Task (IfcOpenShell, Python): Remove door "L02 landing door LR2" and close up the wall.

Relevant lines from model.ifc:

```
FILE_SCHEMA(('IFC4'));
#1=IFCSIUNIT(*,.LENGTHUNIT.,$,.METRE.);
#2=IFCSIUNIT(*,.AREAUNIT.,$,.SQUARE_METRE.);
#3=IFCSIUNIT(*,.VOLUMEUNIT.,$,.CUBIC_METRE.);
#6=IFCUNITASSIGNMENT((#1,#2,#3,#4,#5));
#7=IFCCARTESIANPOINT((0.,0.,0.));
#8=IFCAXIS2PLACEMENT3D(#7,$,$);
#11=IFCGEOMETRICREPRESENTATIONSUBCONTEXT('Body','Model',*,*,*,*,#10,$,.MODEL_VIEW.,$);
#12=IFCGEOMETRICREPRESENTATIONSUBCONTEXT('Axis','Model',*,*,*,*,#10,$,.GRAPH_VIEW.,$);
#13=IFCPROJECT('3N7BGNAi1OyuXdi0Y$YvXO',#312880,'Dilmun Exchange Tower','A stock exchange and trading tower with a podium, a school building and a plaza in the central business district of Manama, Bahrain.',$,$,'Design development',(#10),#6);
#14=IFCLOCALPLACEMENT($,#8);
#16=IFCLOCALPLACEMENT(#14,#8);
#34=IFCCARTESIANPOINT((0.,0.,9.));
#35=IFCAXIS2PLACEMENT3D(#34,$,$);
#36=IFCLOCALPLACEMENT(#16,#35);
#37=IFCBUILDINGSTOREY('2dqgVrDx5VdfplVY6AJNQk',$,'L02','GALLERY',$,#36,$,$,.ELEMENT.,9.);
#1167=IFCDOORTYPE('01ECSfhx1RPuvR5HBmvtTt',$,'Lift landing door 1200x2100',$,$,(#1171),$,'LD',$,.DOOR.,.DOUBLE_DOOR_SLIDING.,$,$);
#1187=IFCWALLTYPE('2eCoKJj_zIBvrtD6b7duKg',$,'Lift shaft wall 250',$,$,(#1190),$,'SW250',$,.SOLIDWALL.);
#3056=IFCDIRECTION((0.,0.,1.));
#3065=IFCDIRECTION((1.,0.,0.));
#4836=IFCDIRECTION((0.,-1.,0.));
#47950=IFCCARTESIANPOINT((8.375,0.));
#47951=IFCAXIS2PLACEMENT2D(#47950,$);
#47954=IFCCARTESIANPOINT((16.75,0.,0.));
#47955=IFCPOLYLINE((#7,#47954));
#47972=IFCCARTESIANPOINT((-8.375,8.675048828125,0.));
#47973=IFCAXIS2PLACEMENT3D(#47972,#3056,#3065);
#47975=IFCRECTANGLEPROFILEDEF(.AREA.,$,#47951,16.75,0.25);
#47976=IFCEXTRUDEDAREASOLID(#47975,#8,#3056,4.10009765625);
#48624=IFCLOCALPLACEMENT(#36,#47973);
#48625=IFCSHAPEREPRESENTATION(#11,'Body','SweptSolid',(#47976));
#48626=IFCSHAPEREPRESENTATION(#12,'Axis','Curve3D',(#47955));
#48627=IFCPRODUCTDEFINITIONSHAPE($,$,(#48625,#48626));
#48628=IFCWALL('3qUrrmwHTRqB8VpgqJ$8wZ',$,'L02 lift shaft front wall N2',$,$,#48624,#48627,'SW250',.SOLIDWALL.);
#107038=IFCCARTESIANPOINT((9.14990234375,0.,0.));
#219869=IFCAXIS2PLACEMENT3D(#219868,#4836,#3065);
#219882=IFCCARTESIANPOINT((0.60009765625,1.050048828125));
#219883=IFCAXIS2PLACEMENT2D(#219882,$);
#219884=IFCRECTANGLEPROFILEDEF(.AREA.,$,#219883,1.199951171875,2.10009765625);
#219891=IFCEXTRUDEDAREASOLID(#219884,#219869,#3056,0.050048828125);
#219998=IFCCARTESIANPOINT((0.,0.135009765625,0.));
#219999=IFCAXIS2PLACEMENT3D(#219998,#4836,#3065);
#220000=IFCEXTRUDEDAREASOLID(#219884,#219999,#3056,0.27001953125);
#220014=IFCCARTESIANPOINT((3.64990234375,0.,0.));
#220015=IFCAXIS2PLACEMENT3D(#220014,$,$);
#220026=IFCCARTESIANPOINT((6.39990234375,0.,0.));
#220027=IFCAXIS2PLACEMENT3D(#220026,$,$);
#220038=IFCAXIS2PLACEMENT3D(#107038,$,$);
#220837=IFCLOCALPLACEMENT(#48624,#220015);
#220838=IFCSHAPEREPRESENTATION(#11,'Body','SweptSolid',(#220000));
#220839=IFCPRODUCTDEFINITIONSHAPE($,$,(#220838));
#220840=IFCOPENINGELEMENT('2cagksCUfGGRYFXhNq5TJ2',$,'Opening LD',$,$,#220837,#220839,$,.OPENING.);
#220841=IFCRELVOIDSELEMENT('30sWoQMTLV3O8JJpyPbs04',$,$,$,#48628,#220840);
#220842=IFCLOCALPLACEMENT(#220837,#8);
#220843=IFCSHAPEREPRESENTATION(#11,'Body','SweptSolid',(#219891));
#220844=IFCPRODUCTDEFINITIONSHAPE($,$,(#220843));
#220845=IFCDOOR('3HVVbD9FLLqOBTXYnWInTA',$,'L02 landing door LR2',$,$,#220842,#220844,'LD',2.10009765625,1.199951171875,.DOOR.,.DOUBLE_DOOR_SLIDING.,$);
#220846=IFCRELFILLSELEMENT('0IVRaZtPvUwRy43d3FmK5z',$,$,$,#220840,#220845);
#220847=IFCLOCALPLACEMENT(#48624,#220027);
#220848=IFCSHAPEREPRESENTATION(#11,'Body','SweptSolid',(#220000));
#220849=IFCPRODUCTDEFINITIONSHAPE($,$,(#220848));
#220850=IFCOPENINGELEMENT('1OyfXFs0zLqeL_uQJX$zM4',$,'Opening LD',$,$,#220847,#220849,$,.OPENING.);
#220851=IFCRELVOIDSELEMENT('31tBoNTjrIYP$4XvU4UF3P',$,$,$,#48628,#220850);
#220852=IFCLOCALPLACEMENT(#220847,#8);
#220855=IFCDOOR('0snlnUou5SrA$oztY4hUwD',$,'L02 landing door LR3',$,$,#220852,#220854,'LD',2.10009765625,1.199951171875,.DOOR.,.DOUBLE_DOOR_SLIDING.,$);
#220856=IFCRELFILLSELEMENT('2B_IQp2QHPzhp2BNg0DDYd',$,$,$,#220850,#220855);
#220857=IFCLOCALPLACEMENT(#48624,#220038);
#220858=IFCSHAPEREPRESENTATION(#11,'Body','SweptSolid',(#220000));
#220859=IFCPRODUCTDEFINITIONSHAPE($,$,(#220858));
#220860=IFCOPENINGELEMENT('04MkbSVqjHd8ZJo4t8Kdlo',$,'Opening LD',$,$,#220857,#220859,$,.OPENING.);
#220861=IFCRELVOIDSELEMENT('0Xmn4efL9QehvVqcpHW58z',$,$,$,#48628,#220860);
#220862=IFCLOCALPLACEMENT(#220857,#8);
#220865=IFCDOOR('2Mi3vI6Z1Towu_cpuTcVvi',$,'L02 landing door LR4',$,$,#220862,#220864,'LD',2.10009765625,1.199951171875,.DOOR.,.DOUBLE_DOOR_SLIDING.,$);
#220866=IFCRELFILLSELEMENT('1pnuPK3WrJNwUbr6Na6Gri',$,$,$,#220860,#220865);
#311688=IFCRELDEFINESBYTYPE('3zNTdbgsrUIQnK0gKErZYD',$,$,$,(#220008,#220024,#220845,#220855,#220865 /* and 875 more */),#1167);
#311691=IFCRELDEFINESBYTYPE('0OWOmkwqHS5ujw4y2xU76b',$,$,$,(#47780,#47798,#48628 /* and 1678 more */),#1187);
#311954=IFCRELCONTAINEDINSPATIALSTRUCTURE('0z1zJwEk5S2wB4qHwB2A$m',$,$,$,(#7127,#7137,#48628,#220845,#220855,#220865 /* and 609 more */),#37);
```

```python
import ifcopenshell
import ifcopenshell.api.feature
import ifcopenshell.api.root
import ifcopenshell.geom
import ifcopenshell.util.shape

model = ifcopenshell.open("model.ifc")
settings = ifcopenshell.geom.settings()


def volume(element):
    """Net volume in cubic metres, openings subtracted."""
    shape = ifcopenshell.geom.create_shape(settings, element)
    return ifcopenshell.util.shape.get_volume(shape.geometry)


door = model.by_guid("3HVVbD9FLLqOBTXYnWInTA")
opening = door.FillsVoids[0].RelatingOpeningElement
wall = opening.VoidsElements[0].RelatingBuildingElement
before = volume(wall)

ifcopenshell.api.root.remove_product(model, product=door)
ifcopenshell.api.feature.remove_feature(model, feature=opening)

after = volume(wall)

print(f"wall volume {before:.3f} -> {after:.3f} m3")

model.write("model_edited.ifc")
```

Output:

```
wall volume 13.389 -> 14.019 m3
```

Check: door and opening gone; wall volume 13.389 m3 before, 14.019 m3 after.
